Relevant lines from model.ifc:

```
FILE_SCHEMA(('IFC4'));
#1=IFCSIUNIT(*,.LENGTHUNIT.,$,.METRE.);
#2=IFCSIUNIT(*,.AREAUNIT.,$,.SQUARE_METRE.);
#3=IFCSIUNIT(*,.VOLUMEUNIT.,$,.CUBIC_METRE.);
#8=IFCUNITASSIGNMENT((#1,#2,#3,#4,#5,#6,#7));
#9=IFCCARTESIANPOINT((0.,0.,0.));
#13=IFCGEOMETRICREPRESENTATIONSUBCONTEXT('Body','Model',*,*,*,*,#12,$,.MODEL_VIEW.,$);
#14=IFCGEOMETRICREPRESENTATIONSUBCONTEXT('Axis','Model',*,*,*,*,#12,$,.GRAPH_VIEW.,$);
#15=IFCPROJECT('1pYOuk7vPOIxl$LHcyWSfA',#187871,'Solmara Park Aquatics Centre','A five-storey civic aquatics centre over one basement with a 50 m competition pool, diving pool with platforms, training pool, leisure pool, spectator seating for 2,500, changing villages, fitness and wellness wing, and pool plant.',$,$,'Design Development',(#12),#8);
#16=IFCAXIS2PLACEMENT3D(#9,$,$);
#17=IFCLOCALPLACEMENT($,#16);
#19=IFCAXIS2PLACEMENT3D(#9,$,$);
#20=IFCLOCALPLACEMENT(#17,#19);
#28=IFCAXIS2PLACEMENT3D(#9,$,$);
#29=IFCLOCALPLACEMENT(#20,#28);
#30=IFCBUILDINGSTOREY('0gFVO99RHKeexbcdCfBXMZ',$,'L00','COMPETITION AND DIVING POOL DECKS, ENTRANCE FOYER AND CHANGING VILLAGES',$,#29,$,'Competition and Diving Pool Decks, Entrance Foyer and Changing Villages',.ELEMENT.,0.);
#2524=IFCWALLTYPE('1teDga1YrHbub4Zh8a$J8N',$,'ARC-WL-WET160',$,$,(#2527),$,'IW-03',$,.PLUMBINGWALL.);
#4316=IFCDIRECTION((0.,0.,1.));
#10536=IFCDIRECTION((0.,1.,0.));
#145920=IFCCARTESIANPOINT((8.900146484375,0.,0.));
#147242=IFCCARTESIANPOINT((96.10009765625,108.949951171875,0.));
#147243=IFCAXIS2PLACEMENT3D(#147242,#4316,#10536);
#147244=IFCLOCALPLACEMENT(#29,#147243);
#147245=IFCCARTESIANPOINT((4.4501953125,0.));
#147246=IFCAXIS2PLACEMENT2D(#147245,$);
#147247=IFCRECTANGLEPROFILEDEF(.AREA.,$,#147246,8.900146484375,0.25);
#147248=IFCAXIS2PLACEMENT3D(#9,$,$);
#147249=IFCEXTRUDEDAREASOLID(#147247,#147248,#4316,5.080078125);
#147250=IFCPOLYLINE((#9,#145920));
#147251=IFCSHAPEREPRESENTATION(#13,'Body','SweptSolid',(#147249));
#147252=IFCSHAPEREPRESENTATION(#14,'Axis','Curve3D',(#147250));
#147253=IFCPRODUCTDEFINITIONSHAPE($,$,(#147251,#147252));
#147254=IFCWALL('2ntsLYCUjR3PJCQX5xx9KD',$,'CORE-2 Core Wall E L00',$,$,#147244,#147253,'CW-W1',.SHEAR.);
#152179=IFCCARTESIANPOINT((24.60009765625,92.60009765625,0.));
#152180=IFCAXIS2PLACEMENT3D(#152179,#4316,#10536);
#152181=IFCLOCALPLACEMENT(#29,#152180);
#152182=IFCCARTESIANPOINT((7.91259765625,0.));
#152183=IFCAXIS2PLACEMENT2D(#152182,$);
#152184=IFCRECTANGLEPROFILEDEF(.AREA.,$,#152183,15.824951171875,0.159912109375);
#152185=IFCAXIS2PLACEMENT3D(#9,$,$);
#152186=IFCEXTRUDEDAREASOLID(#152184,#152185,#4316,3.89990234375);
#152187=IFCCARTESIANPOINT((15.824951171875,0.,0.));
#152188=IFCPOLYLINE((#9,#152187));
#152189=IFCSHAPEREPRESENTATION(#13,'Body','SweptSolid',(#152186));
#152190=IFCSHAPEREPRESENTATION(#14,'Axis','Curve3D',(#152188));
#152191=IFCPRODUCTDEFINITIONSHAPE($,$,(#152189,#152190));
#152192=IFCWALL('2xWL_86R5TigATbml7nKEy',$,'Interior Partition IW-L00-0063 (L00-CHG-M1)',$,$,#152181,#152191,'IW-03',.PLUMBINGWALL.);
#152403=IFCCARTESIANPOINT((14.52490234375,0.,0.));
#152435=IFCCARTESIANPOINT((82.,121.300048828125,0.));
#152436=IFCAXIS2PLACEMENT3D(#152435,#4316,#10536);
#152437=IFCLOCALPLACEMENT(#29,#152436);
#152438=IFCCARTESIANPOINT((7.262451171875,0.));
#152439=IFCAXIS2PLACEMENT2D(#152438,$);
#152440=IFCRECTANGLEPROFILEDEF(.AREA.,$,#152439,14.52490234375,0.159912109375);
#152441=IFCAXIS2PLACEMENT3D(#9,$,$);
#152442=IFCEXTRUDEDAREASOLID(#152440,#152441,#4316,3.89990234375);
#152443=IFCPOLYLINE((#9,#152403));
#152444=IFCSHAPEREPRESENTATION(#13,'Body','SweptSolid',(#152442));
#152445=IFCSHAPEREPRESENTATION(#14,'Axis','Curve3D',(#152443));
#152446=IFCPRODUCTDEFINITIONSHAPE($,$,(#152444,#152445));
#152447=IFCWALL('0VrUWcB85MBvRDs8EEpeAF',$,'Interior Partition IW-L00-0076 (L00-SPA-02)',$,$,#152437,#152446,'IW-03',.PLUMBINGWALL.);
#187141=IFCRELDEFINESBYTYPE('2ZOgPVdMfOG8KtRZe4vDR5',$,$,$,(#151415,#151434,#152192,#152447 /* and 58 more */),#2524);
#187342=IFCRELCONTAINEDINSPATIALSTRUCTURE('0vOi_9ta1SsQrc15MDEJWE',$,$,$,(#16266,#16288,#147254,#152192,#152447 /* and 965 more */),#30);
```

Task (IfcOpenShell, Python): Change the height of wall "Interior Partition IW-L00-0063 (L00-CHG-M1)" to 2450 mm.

```python
import ifcopenshell
import ifcopenshell.geom
import ifcopenshell.util.representation
import ifcopenshell.util.shape
import ifcopenshell.util.unit

model = ifcopenshell.open("model.ifc")
unit_scale = ifcopenshell.util.unit.calculate_unit_scale(model)
settings = ifcopenshell.geom.settings()


def volume(element):
    """Net volume in cubic metres, openings subtracted."""
    shape = ifcopenshell.geom.create_shape(settings, element)
    return ifcopenshell.util.shape.get_volume(shape.geometry)


wall = model.by_guid("2xWL_86R5TigATbml7nKEy")
before = volume(wall)

body = ifcopenshell.util.representation.get_representation(wall, "Model", "Body")
solid = body.Items[0]
old_height = solid.Depth
solid.Depth = 2.45 / unit_scale
after = volume(wall)

print(f"height {old_height:g} -> {solid.Depth:g}, volume {before:.3f} -> {after:.3f} m3")

model.write("model-out.ifc")
```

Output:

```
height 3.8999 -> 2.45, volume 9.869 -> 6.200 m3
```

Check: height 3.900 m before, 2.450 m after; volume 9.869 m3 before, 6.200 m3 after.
